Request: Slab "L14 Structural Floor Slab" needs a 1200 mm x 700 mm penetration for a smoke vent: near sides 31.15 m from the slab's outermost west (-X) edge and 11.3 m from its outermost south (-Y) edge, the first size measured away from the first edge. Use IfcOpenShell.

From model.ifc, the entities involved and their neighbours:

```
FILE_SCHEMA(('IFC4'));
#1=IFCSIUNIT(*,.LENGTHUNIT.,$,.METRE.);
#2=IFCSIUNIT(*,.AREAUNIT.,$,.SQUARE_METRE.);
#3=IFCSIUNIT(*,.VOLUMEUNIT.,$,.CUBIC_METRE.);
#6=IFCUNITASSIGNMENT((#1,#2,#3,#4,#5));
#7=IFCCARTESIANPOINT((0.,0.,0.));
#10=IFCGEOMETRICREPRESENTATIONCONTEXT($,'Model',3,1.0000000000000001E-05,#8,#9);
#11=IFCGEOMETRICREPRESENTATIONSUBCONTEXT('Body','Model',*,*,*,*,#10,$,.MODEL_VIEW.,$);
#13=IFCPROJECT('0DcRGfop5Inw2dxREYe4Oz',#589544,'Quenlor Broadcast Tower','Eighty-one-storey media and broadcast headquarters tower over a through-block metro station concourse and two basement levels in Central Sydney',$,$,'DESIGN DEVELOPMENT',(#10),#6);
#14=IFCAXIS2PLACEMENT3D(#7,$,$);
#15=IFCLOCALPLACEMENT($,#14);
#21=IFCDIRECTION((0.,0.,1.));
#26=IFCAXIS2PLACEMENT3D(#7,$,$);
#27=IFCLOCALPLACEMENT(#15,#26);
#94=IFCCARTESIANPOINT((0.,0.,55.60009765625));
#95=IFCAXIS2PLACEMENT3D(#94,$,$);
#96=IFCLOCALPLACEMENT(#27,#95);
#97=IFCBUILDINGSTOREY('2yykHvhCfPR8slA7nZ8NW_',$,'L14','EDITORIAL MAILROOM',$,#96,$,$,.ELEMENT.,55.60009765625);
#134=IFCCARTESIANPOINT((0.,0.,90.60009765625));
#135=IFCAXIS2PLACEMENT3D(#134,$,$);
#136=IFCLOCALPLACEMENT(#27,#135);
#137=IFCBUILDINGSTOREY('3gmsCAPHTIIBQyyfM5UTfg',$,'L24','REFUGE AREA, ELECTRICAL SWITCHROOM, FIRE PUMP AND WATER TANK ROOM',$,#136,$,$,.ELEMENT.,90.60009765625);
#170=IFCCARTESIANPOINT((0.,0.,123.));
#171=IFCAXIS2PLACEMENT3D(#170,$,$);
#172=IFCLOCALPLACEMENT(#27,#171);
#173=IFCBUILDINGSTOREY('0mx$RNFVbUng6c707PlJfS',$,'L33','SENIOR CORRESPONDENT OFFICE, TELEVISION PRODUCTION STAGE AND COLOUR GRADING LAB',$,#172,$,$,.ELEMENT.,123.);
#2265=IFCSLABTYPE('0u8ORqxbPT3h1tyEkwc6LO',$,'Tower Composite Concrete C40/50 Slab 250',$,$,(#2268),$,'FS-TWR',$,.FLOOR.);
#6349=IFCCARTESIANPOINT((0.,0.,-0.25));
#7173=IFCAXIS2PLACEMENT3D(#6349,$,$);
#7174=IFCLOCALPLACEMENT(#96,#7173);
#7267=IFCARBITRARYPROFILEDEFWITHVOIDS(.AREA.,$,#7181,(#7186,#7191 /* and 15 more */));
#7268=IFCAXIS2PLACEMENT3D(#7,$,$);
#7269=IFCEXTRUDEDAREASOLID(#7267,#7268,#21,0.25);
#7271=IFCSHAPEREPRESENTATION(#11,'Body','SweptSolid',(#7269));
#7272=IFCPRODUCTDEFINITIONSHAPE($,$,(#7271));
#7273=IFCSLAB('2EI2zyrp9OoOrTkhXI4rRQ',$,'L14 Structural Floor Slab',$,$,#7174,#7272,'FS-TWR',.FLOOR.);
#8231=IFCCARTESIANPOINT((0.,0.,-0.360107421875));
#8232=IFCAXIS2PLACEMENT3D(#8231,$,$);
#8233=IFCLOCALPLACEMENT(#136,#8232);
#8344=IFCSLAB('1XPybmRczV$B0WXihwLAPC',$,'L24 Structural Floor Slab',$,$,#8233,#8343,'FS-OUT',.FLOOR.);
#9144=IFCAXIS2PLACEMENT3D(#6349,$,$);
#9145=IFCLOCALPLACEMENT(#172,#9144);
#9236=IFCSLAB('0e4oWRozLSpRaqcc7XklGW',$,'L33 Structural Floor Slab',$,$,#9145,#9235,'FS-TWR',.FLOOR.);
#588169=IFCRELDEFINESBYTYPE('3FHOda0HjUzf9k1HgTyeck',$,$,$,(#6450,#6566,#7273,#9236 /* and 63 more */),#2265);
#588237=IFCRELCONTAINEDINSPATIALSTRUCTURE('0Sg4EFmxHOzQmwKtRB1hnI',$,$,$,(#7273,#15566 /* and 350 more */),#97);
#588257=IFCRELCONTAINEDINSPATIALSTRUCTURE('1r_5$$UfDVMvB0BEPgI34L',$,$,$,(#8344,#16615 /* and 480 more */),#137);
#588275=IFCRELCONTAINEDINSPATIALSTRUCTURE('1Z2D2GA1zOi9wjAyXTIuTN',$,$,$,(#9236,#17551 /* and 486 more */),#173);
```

```python
import numpy as np
import ifcopenshell
import ifcopenshell.api.feature
import ifcopenshell.api.geometry
import ifcopenshell.api.root
import ifcopenshell.geom
import ifcopenshell.util.placement
import ifcopenshell.util.representation
import ifcopenshell.util.shape
import ifcopenshell.util.unit

model = ifcopenshell.open("model.ifc")
unit_scale = ifcopenshell.util.unit.calculate_unit_scale(model)
settings = ifcopenshell.geom.settings()


def volume(element):
    """Net volume in cubic metres, openings subtracted."""
    shape = ifcopenshell.geom.create_shape(settings, element)
    return ifcopenshell.util.shape.get_volume(shape.geometry)


slab = model.by_guid("2EI2zyrp9OoOrTkhXI4rRQ")
before = volume(slab)

# Extent in the slab's own axes, in metres. The edges named are its -X and -Y sides.
slab_shape = ifcopenshell.geom.create_shape(settings, slab)
vertices = ifcopenshell.util.shape.get_vertices(slab_shape.geometry)
x_min, y_min, bottom = vertices.min(axis=0)
top = vertices[:, 2].max()

opening = ifcopenshell.api.root.create_entity(model, ifc_class="IfcOpeningElement", name="Smoke vent opening", predefined_type="OPENING")
context = ifcopenshell.util.representation.get_context(model, "Model", "Body", "MODEL_VIEW")
width, depth = 1.2, 0.7
outline = [(0.0, 0.0), (width, 0.0), (width, depth), (0.0, depth), (0.0, 0.0)]
# Overshoot both faces by 50 mm so the cut is clean.
shape = ifcopenshell.api.geometry.add_slab_representation(
    model, context=context, depth=top - bottom + 0.1, polyline=outline
)
ifcopenshell.api.geometry.assign_representation(model, product=opening, representation=shape)

matrix = ifcopenshell.util.placement.get_local_placement(slab.ObjectPlacement)
matrix[:, 3] = matrix @ np.append(np.array([x_min + 31.15, y_min + 11.3, bottom - 0.05]) / unit_scale, 1.0)
ifcopenshell.api.geometry.edit_object_placement(model, product=opening, matrix=matrix, is_si=False)
ifcopenshell.api.feature.add_feature(model, feature=opening, element=slab)

after = volume(slab)

print(f"slab volume {before:.3f} -> {after:.3f} m3")

model.write("model_updated.ifc")
```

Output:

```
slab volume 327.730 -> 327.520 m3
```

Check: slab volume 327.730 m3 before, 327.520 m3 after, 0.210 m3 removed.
